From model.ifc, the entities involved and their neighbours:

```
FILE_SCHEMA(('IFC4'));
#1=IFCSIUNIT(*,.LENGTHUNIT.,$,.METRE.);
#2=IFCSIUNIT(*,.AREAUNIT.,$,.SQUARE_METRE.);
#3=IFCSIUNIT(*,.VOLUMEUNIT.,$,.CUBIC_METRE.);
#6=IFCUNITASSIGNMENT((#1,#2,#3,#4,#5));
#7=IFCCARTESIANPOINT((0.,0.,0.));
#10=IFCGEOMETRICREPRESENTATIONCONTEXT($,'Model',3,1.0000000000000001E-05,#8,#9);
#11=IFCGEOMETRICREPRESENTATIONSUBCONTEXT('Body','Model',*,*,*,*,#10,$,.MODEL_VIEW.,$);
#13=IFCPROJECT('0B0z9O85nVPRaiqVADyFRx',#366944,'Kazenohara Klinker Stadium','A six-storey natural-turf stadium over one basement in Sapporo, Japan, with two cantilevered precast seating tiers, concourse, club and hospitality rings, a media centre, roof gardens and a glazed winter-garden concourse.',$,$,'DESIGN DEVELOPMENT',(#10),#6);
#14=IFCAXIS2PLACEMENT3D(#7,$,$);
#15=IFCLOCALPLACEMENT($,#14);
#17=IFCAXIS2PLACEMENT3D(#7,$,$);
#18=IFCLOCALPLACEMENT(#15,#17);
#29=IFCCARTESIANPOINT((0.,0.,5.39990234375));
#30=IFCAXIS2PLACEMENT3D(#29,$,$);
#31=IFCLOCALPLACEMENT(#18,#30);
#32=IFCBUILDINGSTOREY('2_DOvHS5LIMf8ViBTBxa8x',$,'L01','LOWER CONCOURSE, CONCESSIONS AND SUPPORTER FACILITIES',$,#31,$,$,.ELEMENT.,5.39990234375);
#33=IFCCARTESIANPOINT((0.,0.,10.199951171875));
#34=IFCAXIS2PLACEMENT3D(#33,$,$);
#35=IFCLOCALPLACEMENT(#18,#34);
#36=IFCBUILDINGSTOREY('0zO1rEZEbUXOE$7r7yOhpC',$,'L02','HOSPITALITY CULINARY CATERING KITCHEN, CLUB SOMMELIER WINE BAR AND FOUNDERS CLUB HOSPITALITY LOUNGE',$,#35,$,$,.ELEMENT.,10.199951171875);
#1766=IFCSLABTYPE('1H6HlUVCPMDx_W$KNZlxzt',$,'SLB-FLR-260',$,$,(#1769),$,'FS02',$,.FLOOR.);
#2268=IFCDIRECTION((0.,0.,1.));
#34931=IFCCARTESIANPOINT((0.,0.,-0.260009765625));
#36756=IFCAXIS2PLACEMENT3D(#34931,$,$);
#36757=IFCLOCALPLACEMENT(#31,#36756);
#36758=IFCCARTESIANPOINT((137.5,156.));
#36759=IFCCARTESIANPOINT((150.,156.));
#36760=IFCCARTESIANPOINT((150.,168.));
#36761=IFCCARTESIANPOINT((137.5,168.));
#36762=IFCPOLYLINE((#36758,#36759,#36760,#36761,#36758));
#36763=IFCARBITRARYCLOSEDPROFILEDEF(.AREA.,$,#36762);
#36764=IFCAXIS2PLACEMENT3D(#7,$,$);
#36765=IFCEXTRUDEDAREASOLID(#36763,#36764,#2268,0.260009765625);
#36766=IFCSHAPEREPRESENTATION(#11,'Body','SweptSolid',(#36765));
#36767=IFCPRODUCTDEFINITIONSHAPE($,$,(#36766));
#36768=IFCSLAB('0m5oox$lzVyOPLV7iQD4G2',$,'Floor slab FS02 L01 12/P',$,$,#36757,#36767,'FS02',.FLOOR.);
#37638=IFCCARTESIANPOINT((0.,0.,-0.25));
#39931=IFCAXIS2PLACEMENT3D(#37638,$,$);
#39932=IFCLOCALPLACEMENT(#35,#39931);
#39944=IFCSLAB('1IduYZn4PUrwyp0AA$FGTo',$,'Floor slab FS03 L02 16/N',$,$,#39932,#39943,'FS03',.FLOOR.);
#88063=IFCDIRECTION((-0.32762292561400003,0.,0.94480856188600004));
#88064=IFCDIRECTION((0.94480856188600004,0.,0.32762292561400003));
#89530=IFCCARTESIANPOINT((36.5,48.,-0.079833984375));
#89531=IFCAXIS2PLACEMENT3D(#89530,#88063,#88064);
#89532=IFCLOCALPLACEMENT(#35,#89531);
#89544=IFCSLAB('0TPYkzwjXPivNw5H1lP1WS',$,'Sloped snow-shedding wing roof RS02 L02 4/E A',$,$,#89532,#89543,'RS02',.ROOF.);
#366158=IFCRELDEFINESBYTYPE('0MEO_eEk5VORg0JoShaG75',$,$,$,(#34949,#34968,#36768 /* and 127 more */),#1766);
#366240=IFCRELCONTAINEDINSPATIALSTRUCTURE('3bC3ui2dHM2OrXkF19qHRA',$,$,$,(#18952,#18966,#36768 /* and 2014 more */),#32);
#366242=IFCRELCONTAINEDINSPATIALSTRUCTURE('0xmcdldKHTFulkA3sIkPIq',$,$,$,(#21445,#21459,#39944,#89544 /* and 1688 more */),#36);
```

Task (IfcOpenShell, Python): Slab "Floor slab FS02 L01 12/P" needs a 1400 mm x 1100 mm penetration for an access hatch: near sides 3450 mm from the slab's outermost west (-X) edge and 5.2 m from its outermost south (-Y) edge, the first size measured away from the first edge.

```python
import numpy as np
import ifcopenshell
import ifcopenshell.api.feature
import ifcopenshell.api.geometry
import ifcopenshell.api.root
import ifcopenshell.geom
import ifcopenshell.util.placement
import ifcopenshell.util.representation
import ifcopenshell.util.shape
import ifcopenshell.util.unit

model = ifcopenshell.open("model.ifc")
unit_scale = ifcopenshell.util.unit.calculate_unit_scale(model)
settings = ifcopenshell.geom.settings()


def volume(element):
    """Net volume in cubic metres, openings subtracted."""
    shape = ifcopenshell.geom.create_shape(settings, element)
    return ifcopenshell.util.shape.get_volume(shape.geometry)


slab = model.by_guid("0m5oox$lzVyOPLV7iQD4G2")
before = volume(slab)

# Extent in the slab's own axes, in metres. The edges named are its -X and -Y sides.
slab_shape = ifcopenshell.geom.create_shape(settings, slab)
vertices = ifcopenshell.util.shape.get_vertices(slab_shape.geometry)
x_min, y_min, bottom = vertices.min(axis=0)
top = vertices[:, 2].max()

opening = ifcopenshell.api.root.create_entity(model, ifc_class="IfcOpeningElement", name="Access hatch opening", predefined_type="OPENING")
context = ifcopenshell.util.representation.get_context(model, "Model", "Body", "MODEL_VIEW")
width, depth = 1.4, 1.1
outline = [(0.0, 0.0), (width, 0.0), (width, depth), (0.0, depth), (0.0, 0.0)]
# Overshoot both faces by 50 mm so the cut is clean.
shape = ifcopenshell.api.geometry.add_slab_representation(
    model, context=context, depth=top - bottom + 0.1, polyline=outline
)
ifcopenshell.api.geometry.assign_representation(model, product=opening, representation=shape)

matrix = ifcopenshell.util.placement.get_local_placement(slab.ObjectPlacement)
matrix[:, 3] = matrix @ np.append(np.array([x_min + 3.45, y_min + 5.2, bottom - 0.05]) / unit_scale, 1.0)
ifcopenshell.api.geometry.edit_object_placement(model, product=opening, matrix=matrix, is_si=False)
ifcopenshell.api.feature.add_feature(model, feature=opening, element=slab)

after = volume(slab)

print(f"slab volume {before:.3f} -> {after:.3f} m3")

model.write("model_updated.ifc")
```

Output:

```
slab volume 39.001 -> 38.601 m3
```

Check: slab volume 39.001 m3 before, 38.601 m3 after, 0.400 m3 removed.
